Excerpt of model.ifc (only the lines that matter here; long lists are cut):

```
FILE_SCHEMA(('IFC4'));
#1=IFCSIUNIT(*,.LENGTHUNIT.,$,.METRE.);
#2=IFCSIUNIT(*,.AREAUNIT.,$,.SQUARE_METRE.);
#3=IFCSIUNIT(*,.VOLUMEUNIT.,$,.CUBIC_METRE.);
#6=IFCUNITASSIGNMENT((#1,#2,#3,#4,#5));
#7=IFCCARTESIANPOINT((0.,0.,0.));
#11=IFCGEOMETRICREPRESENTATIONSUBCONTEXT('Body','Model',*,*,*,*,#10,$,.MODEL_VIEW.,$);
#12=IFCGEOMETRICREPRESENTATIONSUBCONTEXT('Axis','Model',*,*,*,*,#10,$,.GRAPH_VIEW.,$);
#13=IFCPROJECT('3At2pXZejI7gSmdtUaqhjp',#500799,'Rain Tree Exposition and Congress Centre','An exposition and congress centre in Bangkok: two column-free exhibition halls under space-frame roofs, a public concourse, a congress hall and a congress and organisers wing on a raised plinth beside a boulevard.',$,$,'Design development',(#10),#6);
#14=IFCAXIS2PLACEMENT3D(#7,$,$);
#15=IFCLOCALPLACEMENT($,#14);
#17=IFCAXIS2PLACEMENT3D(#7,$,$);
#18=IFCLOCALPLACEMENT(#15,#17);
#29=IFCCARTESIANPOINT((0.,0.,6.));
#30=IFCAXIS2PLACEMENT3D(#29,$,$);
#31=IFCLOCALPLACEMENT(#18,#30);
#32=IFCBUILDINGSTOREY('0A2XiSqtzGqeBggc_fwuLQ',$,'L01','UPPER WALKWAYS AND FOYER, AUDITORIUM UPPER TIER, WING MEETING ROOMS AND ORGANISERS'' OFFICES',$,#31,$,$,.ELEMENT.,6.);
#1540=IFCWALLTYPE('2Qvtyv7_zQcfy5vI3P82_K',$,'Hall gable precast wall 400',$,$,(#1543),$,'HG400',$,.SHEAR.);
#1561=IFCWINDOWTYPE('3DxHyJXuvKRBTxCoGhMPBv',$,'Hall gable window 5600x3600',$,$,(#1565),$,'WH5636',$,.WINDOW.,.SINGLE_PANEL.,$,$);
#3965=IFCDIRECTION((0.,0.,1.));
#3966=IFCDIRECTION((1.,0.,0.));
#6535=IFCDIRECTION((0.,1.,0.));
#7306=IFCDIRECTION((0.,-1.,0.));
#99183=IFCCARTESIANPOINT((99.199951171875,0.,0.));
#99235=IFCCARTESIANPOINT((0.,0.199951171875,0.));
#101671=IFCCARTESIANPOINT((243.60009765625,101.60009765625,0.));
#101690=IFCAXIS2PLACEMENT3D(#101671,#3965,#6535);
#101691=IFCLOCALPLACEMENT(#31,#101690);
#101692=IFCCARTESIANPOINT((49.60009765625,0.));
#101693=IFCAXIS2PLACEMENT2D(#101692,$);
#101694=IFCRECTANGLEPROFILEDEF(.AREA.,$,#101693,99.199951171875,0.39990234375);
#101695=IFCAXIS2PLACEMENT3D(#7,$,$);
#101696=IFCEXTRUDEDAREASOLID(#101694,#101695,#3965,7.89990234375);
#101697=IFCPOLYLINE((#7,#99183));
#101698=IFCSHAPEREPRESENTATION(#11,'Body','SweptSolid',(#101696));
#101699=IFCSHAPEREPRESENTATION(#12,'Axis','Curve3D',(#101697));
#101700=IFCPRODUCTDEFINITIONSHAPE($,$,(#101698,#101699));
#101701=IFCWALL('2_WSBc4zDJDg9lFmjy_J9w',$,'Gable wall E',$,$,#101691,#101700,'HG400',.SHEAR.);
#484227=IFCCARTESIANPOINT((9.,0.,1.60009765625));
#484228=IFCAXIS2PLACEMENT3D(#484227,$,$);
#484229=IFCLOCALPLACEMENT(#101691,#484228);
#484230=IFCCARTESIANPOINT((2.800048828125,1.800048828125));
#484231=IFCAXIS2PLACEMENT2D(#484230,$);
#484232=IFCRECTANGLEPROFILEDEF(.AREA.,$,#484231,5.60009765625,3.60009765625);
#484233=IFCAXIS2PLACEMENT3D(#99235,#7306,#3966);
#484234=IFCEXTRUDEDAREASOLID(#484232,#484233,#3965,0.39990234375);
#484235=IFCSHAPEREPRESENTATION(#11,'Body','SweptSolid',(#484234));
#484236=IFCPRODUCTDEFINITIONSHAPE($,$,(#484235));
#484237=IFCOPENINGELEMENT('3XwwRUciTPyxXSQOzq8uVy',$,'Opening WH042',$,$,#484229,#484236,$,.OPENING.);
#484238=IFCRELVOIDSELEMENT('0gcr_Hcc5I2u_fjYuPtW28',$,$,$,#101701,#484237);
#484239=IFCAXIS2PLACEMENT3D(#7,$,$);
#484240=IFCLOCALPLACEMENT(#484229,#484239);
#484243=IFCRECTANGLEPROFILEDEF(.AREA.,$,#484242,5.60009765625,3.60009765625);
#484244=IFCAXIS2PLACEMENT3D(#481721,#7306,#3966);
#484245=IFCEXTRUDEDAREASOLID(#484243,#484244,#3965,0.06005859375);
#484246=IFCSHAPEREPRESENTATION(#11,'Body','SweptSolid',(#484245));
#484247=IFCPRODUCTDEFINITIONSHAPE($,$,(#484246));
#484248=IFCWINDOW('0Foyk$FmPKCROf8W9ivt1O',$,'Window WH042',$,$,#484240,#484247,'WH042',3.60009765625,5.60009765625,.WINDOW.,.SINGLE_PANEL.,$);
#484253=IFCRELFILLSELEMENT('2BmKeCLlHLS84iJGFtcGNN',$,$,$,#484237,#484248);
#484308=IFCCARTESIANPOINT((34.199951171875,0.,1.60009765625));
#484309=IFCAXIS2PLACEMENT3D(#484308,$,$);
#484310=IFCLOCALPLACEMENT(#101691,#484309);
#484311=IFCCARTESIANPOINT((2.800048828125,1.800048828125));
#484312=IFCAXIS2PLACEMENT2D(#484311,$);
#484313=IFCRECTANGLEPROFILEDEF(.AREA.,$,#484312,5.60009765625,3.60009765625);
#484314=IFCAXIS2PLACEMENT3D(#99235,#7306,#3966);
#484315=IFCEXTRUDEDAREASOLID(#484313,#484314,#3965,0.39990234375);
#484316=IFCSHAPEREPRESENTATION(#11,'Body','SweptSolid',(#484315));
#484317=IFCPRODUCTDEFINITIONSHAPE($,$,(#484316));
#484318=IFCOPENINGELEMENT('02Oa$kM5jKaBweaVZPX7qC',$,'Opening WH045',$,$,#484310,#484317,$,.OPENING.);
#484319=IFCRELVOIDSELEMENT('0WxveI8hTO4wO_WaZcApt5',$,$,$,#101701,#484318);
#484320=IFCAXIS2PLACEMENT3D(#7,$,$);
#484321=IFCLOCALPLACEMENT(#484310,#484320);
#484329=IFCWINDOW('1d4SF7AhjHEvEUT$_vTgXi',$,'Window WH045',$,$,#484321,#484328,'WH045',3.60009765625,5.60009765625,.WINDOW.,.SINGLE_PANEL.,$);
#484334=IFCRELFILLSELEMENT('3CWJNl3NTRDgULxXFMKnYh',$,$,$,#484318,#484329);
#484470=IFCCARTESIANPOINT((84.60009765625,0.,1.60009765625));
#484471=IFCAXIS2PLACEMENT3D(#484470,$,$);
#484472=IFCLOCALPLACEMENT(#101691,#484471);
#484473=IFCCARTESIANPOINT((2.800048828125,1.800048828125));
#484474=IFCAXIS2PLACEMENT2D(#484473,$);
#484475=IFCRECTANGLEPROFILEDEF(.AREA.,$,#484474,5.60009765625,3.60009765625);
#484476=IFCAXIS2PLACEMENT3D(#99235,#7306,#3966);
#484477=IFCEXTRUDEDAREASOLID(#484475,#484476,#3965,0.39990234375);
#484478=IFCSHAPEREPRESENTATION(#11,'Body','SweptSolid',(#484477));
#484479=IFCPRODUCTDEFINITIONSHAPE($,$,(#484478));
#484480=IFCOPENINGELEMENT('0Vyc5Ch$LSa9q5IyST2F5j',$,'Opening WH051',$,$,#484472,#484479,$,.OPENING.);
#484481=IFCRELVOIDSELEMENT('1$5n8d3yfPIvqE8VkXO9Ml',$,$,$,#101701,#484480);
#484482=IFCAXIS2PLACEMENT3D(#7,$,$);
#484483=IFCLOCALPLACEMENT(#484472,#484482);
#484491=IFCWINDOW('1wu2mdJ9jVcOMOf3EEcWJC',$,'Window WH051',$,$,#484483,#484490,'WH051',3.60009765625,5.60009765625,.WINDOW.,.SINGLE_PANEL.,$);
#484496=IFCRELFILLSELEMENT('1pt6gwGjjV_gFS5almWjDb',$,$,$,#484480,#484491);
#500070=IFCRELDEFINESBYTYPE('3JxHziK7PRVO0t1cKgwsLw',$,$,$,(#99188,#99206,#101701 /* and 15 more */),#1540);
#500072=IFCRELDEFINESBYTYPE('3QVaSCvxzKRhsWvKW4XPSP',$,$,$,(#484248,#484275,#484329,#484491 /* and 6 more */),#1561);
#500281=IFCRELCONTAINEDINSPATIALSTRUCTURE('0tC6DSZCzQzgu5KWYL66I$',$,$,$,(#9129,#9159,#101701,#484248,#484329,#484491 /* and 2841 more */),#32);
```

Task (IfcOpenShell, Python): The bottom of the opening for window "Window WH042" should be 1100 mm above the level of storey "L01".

```python
import numpy as np
import ifcopenshell
import ifcopenshell.api.geometry
import ifcopenshell.geom
import ifcopenshell.util.element
import ifcopenshell.util.placement
import ifcopenshell.util.shape
import ifcopenshell.util.unit

model = ifcopenshell.open("model.ifc")
unit_scale = ifcopenshell.util.unit.calculate_unit_scale(model)

window = model.by_guid("0Foyk$FmPKCROf8W9ivt1O")
opening = window.FillsVoids[0].RelatingOpeningElement
storey = ifcopenshell.util.element.get_container(window, ifc_class="IfcBuildingStorey")
level = ifcopenshell.util.placement.get_local_placement(storey.ObjectPlacement)[2, 3]

# The opening's origin need not be at the sill, so measure its lowest point.
shape = ifcopenshell.geom.create_shape(ifcopenshell.geom.settings(), opening)
bottom = ifcopenshell.util.shape.get_shape_bottom_elevation(shape, shape.geometry) / unit_scale
dz = level + 1.1 / unit_scale - bottom

shift = np.array([0.0, 0.0, dz])
# The window is placed relative to its opening, so it follows when the opening moves.
matrix = ifcopenshell.util.placement.get_local_placement(opening.ObjectPlacement)
matrix[:3, 3] += shift
ifcopenshell.api.geometry.edit_object_placement(
    model, product=opening, matrix=matrix, is_si=False, should_transform_children=True
)

print(f"moved by {dz * unit_scale:+.3f} m")

model.write("model_rev.ifc")
```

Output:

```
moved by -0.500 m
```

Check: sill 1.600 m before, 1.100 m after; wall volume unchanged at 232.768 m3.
